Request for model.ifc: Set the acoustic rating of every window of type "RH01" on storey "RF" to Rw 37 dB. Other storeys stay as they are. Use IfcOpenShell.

First a look at what the model holds.

```python
import ifcopenshell
import ifcopenshell.util.element

model = ifcopenshell.open("model.ifc")
print(model.schema)
storey = next(s for s in model.by_type("IfcBuildingStorey") if s.Name == "RF")
windows = [e for e in ifcopenshell.util.element.get_decomposition(storey) if e.is_a("IfcWindow")]
seen = {}
for e in windows:
    element_type = ifcopenshell.util.element.get_type(e)
    key = (element_type.Name if element_type != e and element_type else None, ifcopenshell.util.element.get_pset(e, "Pset_WindowCommon", "AcousticRating"))
    seen[key] = seen.get(key, 0) + 1
for (name, value), count in sorted(seen.items(), key=str):
    print(count, "x", name, "|", value)
```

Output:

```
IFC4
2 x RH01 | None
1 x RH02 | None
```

```python
import ifcopenshell
import ifcopenshell.api.pset
import ifcopenshell.util.element

model = ifcopenshell.open("model.ifc")

storey = next(s for s in model.by_type("IfcBuildingStorey") if s.Name == "RF")
windows = [e for e in ifcopenshell.util.element.get_decomposition(storey) if e.is_a("IfcWindow")]

count = 0
for e in windows:
    element_type = ifcopenshell.util.element.get_type(e)
    if element_type in (None, e) or element_type.Name != "RH01":
        continue
    # add_pset returns the element's existing set when there is one.
    pset = ifcopenshell.api.pset.add_pset(model, product=e, name="Pset_WindowCommon")
    ifcopenshell.api.pset.edit_pset(model, pset=pset, properties={"AcousticRating": "Rw 37 dB"})
    count += 1

print(count, "windows updated")

model.write("model_updated.ifc")
```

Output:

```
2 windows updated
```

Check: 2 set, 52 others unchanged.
